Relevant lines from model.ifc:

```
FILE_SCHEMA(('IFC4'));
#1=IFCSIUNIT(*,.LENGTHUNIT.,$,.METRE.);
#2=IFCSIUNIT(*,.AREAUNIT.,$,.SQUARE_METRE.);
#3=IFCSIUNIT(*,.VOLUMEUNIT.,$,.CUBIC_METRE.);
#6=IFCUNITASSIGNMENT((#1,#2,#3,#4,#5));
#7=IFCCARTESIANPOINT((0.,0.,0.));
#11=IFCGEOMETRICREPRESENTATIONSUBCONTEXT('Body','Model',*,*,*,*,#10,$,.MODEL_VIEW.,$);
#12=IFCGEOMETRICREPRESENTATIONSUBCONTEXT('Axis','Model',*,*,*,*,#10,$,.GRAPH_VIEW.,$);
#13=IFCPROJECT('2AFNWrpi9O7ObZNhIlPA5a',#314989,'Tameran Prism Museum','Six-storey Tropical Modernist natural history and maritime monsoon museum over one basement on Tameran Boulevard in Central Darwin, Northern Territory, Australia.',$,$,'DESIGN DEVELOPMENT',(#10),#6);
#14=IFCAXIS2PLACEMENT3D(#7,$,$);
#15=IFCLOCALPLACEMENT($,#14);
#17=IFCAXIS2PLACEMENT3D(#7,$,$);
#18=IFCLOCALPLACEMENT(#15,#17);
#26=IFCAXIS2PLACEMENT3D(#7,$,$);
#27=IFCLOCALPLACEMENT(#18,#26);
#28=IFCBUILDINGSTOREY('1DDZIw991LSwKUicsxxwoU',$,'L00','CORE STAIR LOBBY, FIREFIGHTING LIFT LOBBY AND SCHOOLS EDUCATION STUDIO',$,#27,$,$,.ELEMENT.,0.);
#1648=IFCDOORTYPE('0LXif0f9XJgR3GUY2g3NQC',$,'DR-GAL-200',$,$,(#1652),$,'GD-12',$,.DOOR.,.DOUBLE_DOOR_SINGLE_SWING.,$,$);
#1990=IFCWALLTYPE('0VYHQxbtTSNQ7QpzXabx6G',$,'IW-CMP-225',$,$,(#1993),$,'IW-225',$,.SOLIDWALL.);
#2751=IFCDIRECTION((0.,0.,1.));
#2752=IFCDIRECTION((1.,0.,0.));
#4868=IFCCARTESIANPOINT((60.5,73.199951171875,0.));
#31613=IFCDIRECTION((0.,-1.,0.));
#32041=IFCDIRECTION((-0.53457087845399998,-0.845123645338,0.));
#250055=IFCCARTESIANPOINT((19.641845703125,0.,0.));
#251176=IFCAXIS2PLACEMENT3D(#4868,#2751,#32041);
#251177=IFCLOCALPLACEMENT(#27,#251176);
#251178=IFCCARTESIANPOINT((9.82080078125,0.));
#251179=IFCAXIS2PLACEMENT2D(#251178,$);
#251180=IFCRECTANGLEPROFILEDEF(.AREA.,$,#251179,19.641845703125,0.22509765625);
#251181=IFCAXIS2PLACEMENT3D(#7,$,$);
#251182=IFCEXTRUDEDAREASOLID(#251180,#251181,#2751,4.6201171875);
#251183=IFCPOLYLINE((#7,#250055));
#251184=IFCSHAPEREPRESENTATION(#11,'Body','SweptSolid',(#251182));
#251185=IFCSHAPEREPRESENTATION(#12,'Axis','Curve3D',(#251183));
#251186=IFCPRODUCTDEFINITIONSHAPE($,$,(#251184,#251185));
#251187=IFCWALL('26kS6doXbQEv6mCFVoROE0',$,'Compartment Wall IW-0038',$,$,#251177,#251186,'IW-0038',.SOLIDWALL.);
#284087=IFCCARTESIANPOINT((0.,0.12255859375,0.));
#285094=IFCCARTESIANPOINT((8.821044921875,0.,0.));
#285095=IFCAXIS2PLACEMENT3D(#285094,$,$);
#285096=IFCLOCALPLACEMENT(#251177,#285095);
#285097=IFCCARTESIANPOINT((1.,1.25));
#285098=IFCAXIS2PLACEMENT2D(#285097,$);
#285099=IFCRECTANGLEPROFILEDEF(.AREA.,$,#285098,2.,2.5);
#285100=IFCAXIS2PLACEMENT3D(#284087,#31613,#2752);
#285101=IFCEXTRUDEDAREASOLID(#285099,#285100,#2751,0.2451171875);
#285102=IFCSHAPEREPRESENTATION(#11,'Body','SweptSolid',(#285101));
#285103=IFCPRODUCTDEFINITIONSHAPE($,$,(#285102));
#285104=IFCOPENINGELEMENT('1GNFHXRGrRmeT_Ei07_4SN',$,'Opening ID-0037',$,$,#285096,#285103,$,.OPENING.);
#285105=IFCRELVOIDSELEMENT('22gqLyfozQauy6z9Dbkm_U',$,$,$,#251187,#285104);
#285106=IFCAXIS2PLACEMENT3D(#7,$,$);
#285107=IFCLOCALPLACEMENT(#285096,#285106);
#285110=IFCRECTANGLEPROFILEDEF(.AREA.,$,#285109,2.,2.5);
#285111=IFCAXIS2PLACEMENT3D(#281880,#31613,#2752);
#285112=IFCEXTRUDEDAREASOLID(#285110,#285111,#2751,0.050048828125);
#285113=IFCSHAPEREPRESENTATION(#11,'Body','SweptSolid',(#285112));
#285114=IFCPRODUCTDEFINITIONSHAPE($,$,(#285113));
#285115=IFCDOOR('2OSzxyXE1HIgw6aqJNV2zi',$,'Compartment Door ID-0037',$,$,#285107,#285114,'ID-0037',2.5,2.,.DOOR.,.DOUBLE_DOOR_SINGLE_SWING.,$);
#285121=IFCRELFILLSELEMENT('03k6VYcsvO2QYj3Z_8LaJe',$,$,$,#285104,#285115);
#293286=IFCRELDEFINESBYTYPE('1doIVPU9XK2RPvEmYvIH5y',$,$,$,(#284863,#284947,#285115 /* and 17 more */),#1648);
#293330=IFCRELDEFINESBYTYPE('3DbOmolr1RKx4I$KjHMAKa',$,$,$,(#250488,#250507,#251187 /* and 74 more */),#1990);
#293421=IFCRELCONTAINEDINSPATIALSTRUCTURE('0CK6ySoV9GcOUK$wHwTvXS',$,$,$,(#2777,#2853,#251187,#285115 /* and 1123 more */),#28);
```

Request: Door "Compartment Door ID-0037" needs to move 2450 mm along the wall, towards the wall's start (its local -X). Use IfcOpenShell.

```python
import ifcopenshell
import ifcopenshell.api.geometry
import ifcopenshell.util.placement
import ifcopenshell.util.unit

model = ifcopenshell.open("model.ifc")
unit_scale = ifcopenshell.util.unit.calculate_unit_scale(model)

door = model.by_guid("2OSzxyXE1HIgw6aqJNV2zi")
opening = door.FillsVoids[0].RelatingOpeningElement
wall = opening.VoidsElements[0].RelatingBuildingElement

wall_matrix = ifcopenshell.util.placement.get_local_placement(wall.ObjectPlacement)
shift = wall_matrix[:3, 0] * -2.45 / unit_scale
before = ifcopenshell.util.placement.get_local_placement(door.ObjectPlacement)[:3, 3].copy()

# The door is placed relative to its opening, so it follows when the opening moves.
matrix = ifcopenshell.util.placement.get_local_placement(opening.ObjectPlacement)
matrix[:3, 3] += shift
ifcopenshell.api.geometry.edit_object_placement(
    model, product=opening, matrix=matrix, is_si=False, should_transform_children=True
)

after = ifcopenshell.util.placement.get_local_placement(door.ObjectPlacement)[:3, 3]
print("door moved by", (after - before).round(3) + 0.0)

model.write("model_rev.ifc")
```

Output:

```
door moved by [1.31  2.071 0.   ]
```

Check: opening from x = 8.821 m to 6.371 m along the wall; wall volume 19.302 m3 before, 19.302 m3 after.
